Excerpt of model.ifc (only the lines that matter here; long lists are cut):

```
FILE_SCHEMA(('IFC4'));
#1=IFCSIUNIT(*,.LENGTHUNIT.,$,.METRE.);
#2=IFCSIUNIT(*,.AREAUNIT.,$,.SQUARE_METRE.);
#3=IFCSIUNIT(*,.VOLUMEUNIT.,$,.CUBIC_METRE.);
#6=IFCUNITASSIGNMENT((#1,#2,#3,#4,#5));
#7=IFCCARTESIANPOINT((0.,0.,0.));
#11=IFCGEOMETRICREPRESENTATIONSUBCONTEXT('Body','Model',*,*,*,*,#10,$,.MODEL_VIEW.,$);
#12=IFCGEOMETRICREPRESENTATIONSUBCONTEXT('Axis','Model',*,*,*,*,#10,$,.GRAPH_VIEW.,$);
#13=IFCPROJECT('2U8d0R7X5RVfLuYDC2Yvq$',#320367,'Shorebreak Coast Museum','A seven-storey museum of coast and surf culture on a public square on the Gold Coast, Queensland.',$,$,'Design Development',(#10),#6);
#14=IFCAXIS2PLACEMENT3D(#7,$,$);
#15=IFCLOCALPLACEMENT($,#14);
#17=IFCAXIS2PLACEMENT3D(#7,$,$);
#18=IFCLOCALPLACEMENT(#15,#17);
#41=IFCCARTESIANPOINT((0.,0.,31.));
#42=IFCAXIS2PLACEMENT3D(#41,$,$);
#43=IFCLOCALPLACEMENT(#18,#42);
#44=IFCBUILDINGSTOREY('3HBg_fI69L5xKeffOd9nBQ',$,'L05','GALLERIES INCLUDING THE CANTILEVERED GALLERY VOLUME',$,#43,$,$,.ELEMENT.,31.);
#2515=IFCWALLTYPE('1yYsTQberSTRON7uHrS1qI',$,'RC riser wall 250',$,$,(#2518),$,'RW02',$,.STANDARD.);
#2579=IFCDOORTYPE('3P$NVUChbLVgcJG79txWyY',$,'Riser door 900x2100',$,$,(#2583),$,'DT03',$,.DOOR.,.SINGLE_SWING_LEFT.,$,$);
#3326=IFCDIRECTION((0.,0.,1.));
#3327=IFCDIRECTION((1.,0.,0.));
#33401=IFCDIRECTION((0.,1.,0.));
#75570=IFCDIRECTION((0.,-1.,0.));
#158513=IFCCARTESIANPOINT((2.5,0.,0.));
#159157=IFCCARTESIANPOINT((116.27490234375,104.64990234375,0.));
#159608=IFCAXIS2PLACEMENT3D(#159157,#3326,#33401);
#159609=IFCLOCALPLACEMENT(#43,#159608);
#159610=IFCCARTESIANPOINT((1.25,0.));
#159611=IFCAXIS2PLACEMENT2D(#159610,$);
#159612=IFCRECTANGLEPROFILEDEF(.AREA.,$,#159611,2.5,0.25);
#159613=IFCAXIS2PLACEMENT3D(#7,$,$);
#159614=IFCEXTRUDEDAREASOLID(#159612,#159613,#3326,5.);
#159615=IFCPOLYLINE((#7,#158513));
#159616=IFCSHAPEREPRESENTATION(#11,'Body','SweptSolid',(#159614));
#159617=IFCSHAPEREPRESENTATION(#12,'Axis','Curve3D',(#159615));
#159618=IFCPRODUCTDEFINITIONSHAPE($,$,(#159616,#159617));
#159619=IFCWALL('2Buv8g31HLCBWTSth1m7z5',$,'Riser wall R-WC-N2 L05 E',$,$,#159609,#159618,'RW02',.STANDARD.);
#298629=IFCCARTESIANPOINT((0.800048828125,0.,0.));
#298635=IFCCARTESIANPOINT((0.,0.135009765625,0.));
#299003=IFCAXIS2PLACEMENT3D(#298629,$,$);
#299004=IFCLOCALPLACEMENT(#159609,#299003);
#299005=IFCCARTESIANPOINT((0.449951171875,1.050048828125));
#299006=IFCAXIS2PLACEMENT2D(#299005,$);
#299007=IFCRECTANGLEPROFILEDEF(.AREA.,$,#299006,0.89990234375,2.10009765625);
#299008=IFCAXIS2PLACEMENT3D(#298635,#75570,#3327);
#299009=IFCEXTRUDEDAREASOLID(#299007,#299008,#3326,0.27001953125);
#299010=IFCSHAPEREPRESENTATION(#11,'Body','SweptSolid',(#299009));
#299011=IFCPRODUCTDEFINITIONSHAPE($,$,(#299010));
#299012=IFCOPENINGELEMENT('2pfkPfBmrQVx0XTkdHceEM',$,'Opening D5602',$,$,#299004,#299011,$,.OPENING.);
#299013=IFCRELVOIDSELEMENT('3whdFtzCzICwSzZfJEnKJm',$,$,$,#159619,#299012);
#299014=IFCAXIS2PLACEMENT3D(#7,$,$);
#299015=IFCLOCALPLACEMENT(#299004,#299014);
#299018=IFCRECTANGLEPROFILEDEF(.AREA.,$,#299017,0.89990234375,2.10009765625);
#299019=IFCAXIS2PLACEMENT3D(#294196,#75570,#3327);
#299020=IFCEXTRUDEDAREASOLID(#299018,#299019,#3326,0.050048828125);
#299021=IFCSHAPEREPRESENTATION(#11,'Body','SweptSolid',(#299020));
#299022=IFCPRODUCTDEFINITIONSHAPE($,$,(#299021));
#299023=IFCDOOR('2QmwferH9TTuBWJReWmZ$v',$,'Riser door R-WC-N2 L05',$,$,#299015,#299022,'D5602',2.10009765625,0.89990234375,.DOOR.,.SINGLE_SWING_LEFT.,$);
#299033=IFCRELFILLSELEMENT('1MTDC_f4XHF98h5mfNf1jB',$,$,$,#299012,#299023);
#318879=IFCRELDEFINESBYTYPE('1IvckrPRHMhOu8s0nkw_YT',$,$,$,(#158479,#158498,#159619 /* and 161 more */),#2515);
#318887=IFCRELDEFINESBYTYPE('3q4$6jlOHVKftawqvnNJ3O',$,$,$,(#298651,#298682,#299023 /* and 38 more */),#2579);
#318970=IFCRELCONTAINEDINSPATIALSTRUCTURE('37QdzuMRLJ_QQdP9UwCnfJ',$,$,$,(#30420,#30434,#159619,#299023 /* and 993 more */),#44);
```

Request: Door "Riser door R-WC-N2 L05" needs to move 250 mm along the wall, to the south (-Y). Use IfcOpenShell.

```python
import ifcopenshell
import ifcopenshell.api.geometry
import ifcopenshell.util.placement
import ifcopenshell.util.unit

model = ifcopenshell.open("model.ifc")
unit_scale = ifcopenshell.util.unit.calculate_unit_scale(model)

door = model.by_guid("2QmwferH9TTuBWJReWmZ$v")
opening = door.FillsVoids[0].RelatingOpeningElement
wall = opening.VoidsElements[0].RelatingBuildingElement

wall_matrix = ifcopenshell.util.placement.get_local_placement(wall.ObjectPlacement)
shift = wall_matrix[:3, 0] * -0.25 / unit_scale
before = ifcopenshell.util.placement.get_local_placement(door.ObjectPlacement)[:3, 3].copy()

# The door is placed relative to its opening, so it follows when the opening moves.
matrix = ifcopenshell.util.placement.get_local_placement(opening.ObjectPlacement)
matrix[:3, 3] += shift
ifcopenshell.api.geometry.edit_object_placement(
    model, product=opening, matrix=matrix, is_si=False, should_transform_children=True
)

after = ifcopenshell.util.placement.get_local_placement(door.ObjectPlacement)[:3, 3]
print("door moved by", (after - before).round(3) + 0.0)

model.write("model_updated.ifc")
```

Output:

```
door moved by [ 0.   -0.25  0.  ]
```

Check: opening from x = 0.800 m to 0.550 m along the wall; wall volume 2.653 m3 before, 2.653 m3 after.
